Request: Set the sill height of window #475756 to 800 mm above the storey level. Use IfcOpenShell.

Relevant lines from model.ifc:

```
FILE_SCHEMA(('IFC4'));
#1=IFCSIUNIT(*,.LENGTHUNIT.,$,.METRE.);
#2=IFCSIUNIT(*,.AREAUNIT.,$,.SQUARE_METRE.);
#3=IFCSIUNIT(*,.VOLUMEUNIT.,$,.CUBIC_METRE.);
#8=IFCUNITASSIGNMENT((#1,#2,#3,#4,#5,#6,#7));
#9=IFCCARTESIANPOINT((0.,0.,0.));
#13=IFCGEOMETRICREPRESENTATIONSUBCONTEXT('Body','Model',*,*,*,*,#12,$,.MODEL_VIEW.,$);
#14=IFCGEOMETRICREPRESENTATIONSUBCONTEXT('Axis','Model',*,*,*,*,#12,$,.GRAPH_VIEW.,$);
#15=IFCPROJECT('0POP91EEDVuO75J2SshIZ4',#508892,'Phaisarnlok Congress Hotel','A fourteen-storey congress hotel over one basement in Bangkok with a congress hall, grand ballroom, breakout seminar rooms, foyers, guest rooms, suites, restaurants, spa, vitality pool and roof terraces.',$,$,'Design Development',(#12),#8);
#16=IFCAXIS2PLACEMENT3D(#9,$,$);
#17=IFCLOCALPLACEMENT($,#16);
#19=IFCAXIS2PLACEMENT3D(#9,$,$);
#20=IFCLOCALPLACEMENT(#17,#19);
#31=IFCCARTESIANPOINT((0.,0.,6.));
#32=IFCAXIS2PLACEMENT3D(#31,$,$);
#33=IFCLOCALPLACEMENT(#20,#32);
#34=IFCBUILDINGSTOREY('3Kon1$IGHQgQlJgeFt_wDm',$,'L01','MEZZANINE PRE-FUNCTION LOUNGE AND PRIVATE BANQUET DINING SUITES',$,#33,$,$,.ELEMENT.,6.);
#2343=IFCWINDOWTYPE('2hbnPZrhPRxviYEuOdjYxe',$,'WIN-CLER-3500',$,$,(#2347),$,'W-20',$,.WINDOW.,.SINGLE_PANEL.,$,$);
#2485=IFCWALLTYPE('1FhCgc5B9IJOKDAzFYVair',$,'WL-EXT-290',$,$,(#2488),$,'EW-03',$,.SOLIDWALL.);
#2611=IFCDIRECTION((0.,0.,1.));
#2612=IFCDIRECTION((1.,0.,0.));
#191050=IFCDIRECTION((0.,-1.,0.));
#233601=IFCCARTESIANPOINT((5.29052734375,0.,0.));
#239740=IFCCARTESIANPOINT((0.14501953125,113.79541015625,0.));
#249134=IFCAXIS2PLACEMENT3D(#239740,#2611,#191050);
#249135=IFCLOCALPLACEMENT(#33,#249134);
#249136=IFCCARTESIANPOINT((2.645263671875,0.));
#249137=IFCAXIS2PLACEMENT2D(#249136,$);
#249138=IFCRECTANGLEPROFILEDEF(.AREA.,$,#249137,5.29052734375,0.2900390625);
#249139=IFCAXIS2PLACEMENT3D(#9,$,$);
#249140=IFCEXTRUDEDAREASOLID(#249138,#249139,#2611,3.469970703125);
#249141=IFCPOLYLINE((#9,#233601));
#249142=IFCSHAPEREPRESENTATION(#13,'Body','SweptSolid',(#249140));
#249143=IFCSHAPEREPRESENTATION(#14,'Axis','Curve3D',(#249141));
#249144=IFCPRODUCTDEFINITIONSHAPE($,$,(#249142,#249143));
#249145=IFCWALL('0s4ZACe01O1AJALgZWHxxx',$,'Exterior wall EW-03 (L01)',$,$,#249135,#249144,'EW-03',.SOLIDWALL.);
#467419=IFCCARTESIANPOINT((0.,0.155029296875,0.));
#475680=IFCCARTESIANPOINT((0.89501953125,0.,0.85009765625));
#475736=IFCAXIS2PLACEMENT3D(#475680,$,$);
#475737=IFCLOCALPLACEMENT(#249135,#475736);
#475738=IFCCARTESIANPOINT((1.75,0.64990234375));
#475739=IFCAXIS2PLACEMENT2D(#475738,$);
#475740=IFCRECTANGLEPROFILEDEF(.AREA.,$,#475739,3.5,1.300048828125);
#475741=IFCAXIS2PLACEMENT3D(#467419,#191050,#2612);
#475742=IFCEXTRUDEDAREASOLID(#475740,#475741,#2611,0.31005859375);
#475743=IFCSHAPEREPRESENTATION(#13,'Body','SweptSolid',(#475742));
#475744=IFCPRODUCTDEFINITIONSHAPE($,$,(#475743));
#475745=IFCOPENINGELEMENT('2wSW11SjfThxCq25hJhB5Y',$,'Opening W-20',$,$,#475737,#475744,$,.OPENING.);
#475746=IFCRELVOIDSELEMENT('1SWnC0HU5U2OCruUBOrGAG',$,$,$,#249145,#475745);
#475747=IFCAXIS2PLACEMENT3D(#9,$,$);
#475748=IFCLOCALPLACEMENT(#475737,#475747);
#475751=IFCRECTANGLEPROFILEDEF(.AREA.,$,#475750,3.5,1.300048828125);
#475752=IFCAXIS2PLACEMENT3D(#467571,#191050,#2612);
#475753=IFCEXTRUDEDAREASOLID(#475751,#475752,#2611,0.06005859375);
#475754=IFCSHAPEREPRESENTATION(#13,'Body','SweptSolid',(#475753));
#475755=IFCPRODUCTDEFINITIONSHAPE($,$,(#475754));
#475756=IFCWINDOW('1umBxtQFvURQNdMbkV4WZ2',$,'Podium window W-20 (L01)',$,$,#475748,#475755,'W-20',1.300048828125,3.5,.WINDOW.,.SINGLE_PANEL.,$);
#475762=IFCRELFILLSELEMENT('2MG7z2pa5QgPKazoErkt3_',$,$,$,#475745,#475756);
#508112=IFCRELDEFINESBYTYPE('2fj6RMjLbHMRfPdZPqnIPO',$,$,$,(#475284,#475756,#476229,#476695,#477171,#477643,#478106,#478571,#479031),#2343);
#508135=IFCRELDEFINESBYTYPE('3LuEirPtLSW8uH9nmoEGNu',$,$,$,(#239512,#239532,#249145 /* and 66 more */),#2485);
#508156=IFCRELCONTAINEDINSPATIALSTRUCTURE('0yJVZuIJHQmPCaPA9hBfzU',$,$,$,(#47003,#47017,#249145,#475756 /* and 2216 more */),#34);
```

```python
import numpy as np
import ifcopenshell
import ifcopenshell.api.geometry
import ifcopenshell.geom
import ifcopenshell.util.element
import ifcopenshell.util.placement
import ifcopenshell.util.shape
import ifcopenshell.util.unit

model = ifcopenshell.open("model.ifc")
unit_scale = ifcopenshell.util.unit.calculate_unit_scale(model)

window = model.by_guid("1umBxtQFvURQNdMbkV4WZ2")
opening = window.FillsVoids[0].RelatingOpeningElement
storey = ifcopenshell.util.element.get_container(window, ifc_class="IfcBuildingStorey")
level = ifcopenshell.util.placement.get_local_placement(storey.ObjectPlacement)[2, 3]

# The opening's origin need not be at the sill, so measure its lowest point.
shape = ifcopenshell.geom.create_shape(ifcopenshell.geom.settings(), opening)
bottom = ifcopenshell.util.shape.get_shape_bottom_elevation(shape, shape.geometry) / unit_scale
dz = level + 0.8 / unit_scale - bottom

shift = np.array([0.0, 0.0, dz])
# The window is placed relative to its opening, so it follows when the opening moves.
matrix = ifcopenshell.util.placement.get_local_placement(opening.ObjectPlacement)
matrix[:3, 3] += shift
ifcopenshell.api.geometry.edit_object_placement(
    model, product=opening, matrix=matrix, is_si=False, should_transform_children=True
)

print(f"moved by {dz * unit_scale:+.3f} m")

model.write("model_rev.ifc")
```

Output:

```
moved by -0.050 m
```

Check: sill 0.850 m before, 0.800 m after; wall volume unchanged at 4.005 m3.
